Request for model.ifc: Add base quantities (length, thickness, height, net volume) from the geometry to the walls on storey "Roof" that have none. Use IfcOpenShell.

First a look at what the model holds.

```python
import ifcopenshell
import ifcopenshell.util.element
import ifcopenshell.util.unit

model = ifcopenshell.open("model.ifc")
print(model.schema)
for unit_type in ("LENGTHUNIT", "AREAUNIT", "VOLUMEUNIT"):
    print(unit_type, ifcopenshell.util.unit.calculate_unit_scale(model, unit_type))
storey = next(s for s in model.by_type("IfcBuildingStorey") if s.Name == "Roof")
walls = [e for e in ifcopenshell.util.element.get_decomposition(storey) if e.is_a("IfcWall")]
for e in sorted(walls, key=lambda e: e.id()):
    print(e.id(), e.is_a(), e.Name, list(ifcopenshell.util.element.get_psets(e, qtos_only=True)), sep=" | ")
```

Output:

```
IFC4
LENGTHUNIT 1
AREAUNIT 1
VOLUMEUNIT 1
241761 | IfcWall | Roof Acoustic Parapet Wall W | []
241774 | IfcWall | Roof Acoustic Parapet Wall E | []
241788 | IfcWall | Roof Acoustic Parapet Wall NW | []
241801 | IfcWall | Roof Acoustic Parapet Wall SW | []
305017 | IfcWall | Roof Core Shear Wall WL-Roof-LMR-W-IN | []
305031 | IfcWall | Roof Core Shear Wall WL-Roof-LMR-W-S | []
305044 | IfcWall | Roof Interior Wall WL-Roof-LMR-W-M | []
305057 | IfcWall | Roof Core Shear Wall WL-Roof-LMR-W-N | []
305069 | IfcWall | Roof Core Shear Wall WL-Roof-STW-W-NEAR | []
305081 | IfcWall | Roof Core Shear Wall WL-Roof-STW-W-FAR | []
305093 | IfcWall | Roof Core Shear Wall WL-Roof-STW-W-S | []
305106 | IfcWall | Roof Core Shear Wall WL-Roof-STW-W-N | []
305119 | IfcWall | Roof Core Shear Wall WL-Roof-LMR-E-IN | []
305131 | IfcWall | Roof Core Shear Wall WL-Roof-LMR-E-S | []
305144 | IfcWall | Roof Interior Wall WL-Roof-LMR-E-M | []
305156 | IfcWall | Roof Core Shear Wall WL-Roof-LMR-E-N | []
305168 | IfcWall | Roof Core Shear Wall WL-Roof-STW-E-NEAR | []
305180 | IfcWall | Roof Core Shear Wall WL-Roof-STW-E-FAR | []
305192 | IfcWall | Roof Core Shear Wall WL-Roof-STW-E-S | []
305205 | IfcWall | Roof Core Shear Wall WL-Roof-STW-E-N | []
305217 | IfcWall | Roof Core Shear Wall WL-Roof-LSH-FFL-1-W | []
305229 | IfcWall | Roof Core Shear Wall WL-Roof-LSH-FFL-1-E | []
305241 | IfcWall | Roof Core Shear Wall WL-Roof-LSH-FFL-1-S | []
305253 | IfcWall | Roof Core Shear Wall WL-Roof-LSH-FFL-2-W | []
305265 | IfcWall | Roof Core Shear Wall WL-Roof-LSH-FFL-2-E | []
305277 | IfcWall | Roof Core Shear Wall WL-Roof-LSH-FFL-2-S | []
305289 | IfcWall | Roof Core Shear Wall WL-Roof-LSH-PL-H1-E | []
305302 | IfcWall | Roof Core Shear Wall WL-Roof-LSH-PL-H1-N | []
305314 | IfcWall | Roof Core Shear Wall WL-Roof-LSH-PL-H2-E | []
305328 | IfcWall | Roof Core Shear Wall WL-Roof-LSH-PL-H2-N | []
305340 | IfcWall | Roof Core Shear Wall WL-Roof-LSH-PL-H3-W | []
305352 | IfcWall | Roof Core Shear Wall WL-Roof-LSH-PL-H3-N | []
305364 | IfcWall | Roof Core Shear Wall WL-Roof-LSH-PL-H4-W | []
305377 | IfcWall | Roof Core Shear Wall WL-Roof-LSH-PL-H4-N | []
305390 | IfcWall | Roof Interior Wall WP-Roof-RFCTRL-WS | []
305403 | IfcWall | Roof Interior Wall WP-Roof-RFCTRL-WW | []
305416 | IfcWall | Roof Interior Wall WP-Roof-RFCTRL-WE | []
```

```python
import ifcopenshell
import ifcopenshell.api.pset
import ifcopenshell.geom
import ifcopenshell.util.element
import ifcopenshell.util.shape
import ifcopenshell.util.unit

model = ifcopenshell.open("model.ifc")
unit_scale = ifcopenshell.util.unit.calculate_unit_scale(model)
volume_scale = ifcopenshell.util.unit.calculate_unit_scale(model, "VOLUMEUNIT")
settings = ifcopenshell.geom.settings()

storey = next(s for s in model.by_type("IfcBuildingStorey") if s.Name == "Roof")
walls = [e for e in ifcopenshell.util.element.get_decomposition(storey) if e.is_a("IfcWall")]

for e in sorted(walls, key=lambda e: e.id()):
    if ifcopenshell.util.element.get_psets(e, qtos_only=True, should_inherit=False):
        continue
    # Geometry comes back in metres, in the element's own axes.
    shape = ifcopenshell.geom.create_shape(settings, e)
    values = {
        "Length": ifcopenshell.util.shape.get_x(shape.geometry) / unit_scale,
        "Width": ifcopenshell.util.shape.get_y(shape.geometry) / unit_scale,
        "Height": ifcopenshell.util.shape.get_z(shape.geometry) / unit_scale,
        "NetVolume": ifcopenshell.util.shape.get_volume(shape.geometry) / volume_scale,
    }
    qto = ifcopenshell.api.pset.add_qto(model, product=e, name="Qto_WallBaseQuantities")
    ifcopenshell.api.pset.edit_qto(model, qto=qto, properties=values)
    print(e.id(), {k: round(v, 3) for k, v in values.items()})

model.write("model_rev.ifc")
```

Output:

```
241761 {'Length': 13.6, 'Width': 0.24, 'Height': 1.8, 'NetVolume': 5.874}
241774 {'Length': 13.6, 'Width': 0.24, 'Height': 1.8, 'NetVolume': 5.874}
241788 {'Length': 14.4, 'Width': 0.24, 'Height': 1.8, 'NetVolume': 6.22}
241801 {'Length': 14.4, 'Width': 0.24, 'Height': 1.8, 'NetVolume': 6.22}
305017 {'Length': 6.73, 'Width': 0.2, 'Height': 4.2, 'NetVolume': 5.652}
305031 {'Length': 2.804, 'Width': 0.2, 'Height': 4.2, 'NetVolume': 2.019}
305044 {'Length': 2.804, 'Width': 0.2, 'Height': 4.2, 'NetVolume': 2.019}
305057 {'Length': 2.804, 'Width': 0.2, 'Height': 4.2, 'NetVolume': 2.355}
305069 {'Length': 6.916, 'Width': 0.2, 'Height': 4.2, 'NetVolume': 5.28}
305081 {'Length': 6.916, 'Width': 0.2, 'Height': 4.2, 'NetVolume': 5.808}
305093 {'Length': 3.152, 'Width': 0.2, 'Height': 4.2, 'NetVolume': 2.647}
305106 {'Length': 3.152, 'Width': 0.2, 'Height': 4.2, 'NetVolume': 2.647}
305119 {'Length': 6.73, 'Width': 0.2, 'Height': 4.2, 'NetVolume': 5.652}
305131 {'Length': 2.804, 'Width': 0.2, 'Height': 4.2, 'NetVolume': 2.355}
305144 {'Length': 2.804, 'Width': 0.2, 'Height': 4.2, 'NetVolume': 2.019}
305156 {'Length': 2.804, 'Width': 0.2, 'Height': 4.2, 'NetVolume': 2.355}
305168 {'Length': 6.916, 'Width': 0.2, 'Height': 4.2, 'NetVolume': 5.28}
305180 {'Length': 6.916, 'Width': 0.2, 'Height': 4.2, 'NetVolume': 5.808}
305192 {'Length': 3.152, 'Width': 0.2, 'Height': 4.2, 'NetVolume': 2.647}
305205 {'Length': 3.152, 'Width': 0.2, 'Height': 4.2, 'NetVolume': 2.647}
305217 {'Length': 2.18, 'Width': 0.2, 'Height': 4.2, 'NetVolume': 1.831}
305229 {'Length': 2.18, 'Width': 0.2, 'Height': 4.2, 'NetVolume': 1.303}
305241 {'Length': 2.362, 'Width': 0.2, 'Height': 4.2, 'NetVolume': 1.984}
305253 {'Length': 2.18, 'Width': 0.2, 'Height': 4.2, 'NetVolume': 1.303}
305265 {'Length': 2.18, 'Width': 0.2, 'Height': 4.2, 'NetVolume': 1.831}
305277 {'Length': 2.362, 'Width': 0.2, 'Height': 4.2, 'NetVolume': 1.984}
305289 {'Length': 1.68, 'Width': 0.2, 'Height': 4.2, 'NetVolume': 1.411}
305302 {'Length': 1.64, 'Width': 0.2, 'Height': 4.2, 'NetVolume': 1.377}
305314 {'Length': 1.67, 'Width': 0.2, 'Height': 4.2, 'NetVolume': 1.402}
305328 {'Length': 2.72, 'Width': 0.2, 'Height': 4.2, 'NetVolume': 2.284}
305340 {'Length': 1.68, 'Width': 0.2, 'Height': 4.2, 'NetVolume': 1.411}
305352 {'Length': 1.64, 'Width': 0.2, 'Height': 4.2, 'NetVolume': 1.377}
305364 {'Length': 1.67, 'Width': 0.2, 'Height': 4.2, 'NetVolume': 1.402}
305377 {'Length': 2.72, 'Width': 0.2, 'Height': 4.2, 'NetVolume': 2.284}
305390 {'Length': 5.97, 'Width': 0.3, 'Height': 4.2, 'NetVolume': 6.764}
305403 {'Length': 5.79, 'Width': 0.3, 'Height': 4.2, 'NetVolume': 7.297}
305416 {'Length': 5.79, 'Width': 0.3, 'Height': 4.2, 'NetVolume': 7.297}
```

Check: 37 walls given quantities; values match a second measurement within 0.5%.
